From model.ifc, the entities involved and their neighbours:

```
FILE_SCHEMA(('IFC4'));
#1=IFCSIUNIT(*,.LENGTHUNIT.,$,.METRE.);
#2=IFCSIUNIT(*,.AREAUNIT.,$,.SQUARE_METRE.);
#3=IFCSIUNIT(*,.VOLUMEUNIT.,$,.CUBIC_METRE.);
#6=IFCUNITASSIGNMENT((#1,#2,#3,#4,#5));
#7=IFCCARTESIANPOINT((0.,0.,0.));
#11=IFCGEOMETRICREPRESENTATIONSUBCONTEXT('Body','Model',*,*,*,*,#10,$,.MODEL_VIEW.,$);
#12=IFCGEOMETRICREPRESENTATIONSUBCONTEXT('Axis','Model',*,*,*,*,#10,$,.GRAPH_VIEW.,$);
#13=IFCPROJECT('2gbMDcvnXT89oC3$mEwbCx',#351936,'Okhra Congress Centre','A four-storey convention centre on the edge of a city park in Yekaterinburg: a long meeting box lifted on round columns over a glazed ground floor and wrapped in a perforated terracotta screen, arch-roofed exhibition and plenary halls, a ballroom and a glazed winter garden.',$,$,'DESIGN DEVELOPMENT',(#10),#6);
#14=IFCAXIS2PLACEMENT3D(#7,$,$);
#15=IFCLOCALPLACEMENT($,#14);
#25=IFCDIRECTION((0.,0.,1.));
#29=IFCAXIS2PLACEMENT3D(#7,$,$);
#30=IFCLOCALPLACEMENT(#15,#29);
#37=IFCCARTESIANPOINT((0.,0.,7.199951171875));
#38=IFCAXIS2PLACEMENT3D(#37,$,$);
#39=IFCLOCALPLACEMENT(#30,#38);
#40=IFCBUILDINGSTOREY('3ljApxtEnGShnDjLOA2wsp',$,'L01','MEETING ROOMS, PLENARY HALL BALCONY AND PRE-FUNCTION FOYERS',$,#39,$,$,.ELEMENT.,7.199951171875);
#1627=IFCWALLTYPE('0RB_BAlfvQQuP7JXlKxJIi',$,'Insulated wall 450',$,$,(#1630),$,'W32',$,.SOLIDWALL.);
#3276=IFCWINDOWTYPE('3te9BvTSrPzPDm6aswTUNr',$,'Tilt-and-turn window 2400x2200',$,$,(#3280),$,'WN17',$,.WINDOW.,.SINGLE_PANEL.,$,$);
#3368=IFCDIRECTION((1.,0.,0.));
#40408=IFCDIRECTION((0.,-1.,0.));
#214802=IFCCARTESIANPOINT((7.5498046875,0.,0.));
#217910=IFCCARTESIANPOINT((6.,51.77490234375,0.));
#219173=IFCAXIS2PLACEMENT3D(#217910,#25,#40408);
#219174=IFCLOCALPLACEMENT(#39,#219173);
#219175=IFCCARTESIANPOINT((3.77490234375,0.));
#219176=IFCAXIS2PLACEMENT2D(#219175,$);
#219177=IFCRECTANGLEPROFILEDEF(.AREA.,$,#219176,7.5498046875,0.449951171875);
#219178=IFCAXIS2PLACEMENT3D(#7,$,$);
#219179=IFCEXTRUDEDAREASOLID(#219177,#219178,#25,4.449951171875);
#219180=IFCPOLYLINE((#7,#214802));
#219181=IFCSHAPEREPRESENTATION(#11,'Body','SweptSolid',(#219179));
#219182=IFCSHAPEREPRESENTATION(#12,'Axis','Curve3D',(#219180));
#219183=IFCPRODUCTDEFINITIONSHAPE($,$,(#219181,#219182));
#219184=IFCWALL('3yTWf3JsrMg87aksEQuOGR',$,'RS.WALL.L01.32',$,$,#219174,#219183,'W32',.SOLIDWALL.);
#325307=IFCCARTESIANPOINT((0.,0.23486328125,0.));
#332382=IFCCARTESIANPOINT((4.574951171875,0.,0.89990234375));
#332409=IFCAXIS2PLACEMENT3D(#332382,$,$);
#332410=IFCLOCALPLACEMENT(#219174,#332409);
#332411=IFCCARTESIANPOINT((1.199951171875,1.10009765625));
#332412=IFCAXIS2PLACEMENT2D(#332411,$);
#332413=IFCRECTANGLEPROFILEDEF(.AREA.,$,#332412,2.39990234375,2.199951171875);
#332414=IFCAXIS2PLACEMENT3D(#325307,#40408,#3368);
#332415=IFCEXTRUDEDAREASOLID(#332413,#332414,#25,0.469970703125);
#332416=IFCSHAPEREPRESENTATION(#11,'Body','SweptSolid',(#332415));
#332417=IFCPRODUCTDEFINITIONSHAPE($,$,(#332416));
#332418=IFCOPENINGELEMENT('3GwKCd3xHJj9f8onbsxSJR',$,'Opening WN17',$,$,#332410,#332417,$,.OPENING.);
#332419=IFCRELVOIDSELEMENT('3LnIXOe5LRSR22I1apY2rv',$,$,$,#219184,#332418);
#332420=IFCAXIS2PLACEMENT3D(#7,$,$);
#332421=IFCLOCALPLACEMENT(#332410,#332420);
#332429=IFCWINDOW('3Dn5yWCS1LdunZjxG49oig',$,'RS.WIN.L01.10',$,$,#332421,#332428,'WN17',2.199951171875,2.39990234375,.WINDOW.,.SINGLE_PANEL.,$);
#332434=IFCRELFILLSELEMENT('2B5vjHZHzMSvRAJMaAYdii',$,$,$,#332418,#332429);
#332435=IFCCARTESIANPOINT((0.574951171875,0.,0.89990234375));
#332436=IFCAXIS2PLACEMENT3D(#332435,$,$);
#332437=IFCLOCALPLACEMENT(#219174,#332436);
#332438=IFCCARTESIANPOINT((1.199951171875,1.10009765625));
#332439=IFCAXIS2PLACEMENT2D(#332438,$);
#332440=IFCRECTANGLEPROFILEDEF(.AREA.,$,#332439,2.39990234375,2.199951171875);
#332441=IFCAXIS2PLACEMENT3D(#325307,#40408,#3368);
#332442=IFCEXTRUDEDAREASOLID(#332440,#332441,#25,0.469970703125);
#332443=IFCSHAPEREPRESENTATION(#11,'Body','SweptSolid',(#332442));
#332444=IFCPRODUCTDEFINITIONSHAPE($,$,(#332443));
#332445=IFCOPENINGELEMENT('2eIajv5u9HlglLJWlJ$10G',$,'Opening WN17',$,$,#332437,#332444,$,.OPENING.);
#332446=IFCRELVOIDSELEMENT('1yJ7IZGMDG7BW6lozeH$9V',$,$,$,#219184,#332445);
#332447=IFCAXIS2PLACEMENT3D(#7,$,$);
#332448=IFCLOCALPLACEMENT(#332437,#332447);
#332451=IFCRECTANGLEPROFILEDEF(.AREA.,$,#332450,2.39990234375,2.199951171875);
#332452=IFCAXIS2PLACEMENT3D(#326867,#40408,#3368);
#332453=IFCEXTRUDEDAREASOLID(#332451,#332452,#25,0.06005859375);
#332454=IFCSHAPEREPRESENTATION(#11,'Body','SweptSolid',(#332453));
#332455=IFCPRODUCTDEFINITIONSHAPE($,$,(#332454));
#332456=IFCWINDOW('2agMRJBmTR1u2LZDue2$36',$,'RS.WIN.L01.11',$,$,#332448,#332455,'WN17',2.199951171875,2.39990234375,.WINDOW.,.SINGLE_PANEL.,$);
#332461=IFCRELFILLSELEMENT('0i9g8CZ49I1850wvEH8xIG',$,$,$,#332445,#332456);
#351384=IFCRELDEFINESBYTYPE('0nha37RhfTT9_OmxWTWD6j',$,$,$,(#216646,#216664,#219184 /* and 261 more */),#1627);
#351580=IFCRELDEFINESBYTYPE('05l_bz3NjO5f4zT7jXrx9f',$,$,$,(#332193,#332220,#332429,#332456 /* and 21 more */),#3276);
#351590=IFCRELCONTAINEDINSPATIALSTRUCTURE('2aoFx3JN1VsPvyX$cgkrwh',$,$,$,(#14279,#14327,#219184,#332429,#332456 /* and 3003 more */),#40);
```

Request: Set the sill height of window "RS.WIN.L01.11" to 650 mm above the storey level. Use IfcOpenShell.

```python
import numpy as np
import ifcopenshell
import ifcopenshell.api.geometry
import ifcopenshell.geom
import ifcopenshell.util.element
import ifcopenshell.util.placement
import ifcopenshell.util.shape
import ifcopenshell.util.unit

model = ifcopenshell.open("model.ifc")
unit_scale = ifcopenshell.util.unit.calculate_unit_scale(model)

window = model.by_id(332456)
opening = window.FillsVoids[0].RelatingOpeningElement
storey = ifcopenshell.util.element.get_container(window, ifc_class="IfcBuildingStorey")
level = ifcopenshell.util.placement.get_local_placement(storey.ObjectPlacement)[2, 3]

# The opening's origin need not be at the sill, so measure its lowest point.
shape = ifcopenshell.geom.create_shape(ifcopenshell.geom.settings(), opening)
bottom = ifcopenshell.util.shape.get_shape_bottom_elevation(shape, shape.geometry) / unit_scale
dz = level + 0.65 - bottom

shift = np.array([0.0, 0.0, dz])
# The window is placed relative to its opening, so it follows when the opening moves.
matrix = ifcopenshell.util.placement.get_local_placement(opening.ObjectPlacement)
matrix[:3, 3] += shift
ifcopenshell.api.geometry.edit_object_placement(
    model, product=opening, matrix=matrix, is_si=False, should_transform_children=True
)

print(f"moved by {dz * unit_scale:+.3f} m")

model.write("model_v2.ifc")
```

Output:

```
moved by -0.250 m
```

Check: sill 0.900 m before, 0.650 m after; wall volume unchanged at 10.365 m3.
